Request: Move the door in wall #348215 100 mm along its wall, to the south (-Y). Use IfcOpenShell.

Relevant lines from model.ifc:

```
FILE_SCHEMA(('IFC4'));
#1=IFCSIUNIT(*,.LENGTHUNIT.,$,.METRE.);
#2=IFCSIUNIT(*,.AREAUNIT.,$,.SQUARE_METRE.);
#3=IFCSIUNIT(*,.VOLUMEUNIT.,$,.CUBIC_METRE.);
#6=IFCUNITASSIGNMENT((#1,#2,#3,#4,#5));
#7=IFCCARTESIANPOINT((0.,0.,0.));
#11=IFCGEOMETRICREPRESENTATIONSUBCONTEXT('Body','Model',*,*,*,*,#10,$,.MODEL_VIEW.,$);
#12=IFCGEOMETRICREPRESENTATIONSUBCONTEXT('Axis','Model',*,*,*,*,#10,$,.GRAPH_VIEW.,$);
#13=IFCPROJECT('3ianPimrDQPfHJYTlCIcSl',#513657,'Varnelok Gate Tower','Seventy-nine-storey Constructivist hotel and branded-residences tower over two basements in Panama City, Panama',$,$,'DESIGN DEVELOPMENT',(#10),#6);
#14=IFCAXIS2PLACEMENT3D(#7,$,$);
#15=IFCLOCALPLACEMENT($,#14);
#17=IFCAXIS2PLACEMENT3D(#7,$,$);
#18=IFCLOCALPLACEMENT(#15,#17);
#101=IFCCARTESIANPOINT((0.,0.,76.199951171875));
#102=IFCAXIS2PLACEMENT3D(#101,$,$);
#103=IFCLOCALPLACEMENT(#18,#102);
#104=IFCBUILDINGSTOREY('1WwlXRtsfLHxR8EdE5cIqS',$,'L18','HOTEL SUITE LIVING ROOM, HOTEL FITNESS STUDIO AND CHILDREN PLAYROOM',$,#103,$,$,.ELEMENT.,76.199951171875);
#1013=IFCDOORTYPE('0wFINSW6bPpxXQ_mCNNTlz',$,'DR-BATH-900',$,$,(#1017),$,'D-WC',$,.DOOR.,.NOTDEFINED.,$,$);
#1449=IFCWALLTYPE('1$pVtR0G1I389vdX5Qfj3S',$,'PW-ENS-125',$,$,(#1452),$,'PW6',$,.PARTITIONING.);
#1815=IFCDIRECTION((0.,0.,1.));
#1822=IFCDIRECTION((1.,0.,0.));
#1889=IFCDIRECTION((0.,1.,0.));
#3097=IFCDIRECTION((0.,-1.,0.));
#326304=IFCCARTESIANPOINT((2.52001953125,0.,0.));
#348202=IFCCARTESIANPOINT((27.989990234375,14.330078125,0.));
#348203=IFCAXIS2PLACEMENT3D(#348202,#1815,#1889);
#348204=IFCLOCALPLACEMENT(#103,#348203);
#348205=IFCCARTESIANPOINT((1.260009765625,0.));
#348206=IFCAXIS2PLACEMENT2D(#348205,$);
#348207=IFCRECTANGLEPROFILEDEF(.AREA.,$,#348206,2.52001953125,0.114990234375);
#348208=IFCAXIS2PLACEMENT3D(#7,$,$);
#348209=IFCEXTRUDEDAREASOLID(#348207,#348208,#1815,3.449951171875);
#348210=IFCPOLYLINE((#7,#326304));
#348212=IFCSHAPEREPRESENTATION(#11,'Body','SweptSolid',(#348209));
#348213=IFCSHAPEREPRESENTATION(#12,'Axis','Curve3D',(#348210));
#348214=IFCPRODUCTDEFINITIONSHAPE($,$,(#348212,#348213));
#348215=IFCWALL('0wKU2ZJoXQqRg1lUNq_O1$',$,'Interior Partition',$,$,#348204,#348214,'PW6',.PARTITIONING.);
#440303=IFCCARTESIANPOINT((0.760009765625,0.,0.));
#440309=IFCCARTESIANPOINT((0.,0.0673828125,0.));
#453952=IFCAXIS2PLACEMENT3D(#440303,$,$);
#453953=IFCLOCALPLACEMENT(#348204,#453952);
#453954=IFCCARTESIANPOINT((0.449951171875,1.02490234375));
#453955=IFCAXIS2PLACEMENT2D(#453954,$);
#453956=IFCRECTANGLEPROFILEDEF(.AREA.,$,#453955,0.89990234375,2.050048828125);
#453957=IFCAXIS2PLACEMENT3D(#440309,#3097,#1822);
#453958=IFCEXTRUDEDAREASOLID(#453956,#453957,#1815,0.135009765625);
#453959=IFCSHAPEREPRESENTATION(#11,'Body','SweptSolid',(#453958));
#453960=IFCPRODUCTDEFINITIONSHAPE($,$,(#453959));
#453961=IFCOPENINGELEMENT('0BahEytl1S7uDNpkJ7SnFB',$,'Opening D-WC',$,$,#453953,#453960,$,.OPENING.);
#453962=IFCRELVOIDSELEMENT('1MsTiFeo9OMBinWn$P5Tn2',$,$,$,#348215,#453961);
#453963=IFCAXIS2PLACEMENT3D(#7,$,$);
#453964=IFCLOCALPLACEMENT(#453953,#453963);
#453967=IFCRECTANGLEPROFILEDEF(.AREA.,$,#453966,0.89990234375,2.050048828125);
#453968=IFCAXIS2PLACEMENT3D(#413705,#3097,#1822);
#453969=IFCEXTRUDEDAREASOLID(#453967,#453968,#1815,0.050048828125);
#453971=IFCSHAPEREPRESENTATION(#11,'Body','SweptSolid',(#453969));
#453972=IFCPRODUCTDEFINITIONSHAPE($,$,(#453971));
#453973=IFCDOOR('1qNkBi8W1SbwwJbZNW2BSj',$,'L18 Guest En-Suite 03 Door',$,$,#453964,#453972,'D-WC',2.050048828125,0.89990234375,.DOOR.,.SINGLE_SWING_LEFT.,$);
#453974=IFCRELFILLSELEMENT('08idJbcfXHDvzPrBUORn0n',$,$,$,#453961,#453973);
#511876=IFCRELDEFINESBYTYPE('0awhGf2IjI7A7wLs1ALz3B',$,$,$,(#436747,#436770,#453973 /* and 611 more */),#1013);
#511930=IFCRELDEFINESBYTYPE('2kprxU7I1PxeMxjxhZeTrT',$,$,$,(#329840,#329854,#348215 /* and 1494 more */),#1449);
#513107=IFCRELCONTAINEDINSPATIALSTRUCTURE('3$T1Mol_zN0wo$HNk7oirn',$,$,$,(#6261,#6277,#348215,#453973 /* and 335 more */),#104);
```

```python
import ifcopenshell
import ifcopenshell.api.geometry
import ifcopenshell.util.placement
import ifcopenshell.util.unit

model = ifcopenshell.open("model.ifc")
unit_scale = ifcopenshell.util.unit.calculate_unit_scale(model)

door = model.by_id(453973)
opening = door.FillsVoids[0].RelatingOpeningElement
wall = opening.VoidsElements[0].RelatingBuildingElement

wall_matrix = ifcopenshell.util.placement.get_local_placement(wall.ObjectPlacement)
shift = wall_matrix[:3, 0] * -0.1 / unit_scale
before = ifcopenshell.util.placement.get_local_placement(door.ObjectPlacement)[:3, 3].copy()

# The door is placed relative to its opening, so it follows when the opening moves.
matrix = ifcopenshell.util.placement.get_local_placement(opening.ObjectPlacement)
matrix[:3, 3] += shift
ifcopenshell.api.geometry.edit_object_placement(
    model, product=opening, matrix=matrix, is_si=False, should_transform_children=True
)

after = ifcopenshell.util.placement.get_local_placement(door.ObjectPlacement)[:3, 3]
print("door moved by", (after - before).round(3) + 0.0)

model.write("model_updated.ifc")
```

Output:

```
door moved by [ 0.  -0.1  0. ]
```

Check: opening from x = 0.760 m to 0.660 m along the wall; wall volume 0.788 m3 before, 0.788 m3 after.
